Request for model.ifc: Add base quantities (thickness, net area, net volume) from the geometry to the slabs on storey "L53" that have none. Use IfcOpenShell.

First a look at what the model holds.

```python
import ifcopenshell
import ifcopenshell.util.element
import ifcopenshell.util.unit

model = ifcopenshell.open("model.ifc")
print(model.schema)
for unit_type in ("LENGTHUNIT", "AREAUNIT", "VOLUMEUNIT"):
    print(unit_type, ifcopenshell.util.unit.calculate_unit_scale(model, unit_type))
storey = next(s for s in model.by_type("IfcBuildingStorey") if s.Name == "L53")
slabs = [e for e in ifcopenshell.util.element.get_decomposition(storey) if e.is_a("IfcSlab")]
for e in sorted(slabs, key=lambda e: e.id()):
    print(e.id(), e.is_a(), e.Name, list(ifcopenshell.util.element.get_psets(e, qtos_only=True)), sep=" | ")
```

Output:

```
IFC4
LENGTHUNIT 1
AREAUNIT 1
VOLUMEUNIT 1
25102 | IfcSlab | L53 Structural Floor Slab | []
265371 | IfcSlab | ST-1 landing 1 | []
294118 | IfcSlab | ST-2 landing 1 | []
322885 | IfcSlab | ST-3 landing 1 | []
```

```python
import ifcopenshell
import ifcopenshell.api.pset
import ifcopenshell.geom
import ifcopenshell.util.element
import ifcopenshell.util.shape
import ifcopenshell.util.unit

model = ifcopenshell.open("model.ifc")
unit_scale = ifcopenshell.util.unit.calculate_unit_scale(model)
area_scale = ifcopenshell.util.unit.calculate_unit_scale(model, "AREAUNIT")
volume_scale = ifcopenshell.util.unit.calculate_unit_scale(model, "VOLUMEUNIT")
settings = ifcopenshell.geom.settings()

storey = next(s for s in model.by_type("IfcBuildingStorey") if s.Name == "L53")
slabs = [e for e in ifcopenshell.util.element.get_decomposition(storey) if e.is_a("IfcSlab")]

for e in sorted(slabs, key=lambda e: e.id()):
    if ifcopenshell.util.element.get_psets(e, qtos_only=True, should_inherit=False):
        continue
    # Geometry comes back in metres, in the element's own axes.
    shape = ifcopenshell.geom.create_shape(settings, e)
    values = {
        "Width": ifcopenshell.util.shape.get_z(shape.geometry) / unit_scale,
        "NetArea": ifcopenshell.util.shape.get_footprint_area(shape.geometry) / area_scale,
        "NetVolume": ifcopenshell.util.shape.get_volume(shape.geometry) / volume_scale,
    }
    qto = ifcopenshell.api.pset.add_qto(model, product=e, name="Qto_SlabBaseQuantities")
    ifcopenshell.api.pset.edit_qto(model, qto=qto, properties=values)
    print(e.id(), {k: round(v, 3) for k, v in values.items()})

model.write("model-out.ifc")
```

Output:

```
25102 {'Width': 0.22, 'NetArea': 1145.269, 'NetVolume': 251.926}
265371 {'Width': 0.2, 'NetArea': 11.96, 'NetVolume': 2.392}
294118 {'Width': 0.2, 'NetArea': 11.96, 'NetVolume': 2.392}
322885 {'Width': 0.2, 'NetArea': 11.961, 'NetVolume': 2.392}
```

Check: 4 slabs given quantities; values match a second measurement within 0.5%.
